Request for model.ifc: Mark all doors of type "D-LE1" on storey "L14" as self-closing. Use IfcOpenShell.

First a look at what the model holds.

```python
import ifcopenshell
import ifcopenshell.util.element

model = ifcopenshell.open("model.ifc")
print(model.schema)
storey = next(s for s in model.by_type("IfcBuildingStorey") if s.Name == "L14")
doors = [e for e in ifcopenshell.util.element.get_decomposition(storey) if e.is_a("IfcDoor")]
seen = {}
for e in doors:
    element_type = ifcopenshell.util.element.get_type(e)
    key = (element_type.Name if element_type != e and element_type else None, ifcopenshell.util.element.get_pset(e, "Pset_DoorCommon", "SelfClosing"))
    seen[key] = seen.get(key, 0) + 1
for (name, value), count in sorted(seen.items(), key=str):
    print(count, "x", name, "|", value)
```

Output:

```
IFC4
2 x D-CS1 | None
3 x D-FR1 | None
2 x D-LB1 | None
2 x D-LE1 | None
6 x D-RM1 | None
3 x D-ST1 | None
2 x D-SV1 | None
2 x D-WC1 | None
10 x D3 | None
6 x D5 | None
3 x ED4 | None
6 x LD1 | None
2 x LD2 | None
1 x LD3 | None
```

```python
import ifcopenshell
import ifcopenshell.api.pset
import ifcopenshell.util.element

model = ifcopenshell.open("model.ifc")

storey = next(s for s in model.by_type("IfcBuildingStorey") if s.Name == "L14")
doors = [e for e in ifcopenshell.util.element.get_decomposition(storey) if e.is_a("IfcDoor")]

count = 0
for e in doors:
    element_type = ifcopenshell.util.element.get_type(e)
    if element_type in (None, e) or element_type.Name != "D-LE1":
        continue
    found = ifcopenshell.util.element.get_pset(e, "Pset_DoorCommon", should_inherit=False)
    if found:
        pset = model.by_id(found["id"])
        if len(ifcopenshell.util.element.get_elements_by_pset(pset)) > 1:
            pset = ifcopenshell.api.pset.unshare_pset(model, products=[e], pset=pset)[0]
    else:
        pset = ifcopenshell.api.pset.add_pset(model, product=e, name="Pset_DoorCommon")
    ifcopenshell.api.pset.edit_pset(model, pset=pset, properties={"SelfClosing": True})
    count += 1

print(count, "doors updated")

model.write("model_v2.ifc")
```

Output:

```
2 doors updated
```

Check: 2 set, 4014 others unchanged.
